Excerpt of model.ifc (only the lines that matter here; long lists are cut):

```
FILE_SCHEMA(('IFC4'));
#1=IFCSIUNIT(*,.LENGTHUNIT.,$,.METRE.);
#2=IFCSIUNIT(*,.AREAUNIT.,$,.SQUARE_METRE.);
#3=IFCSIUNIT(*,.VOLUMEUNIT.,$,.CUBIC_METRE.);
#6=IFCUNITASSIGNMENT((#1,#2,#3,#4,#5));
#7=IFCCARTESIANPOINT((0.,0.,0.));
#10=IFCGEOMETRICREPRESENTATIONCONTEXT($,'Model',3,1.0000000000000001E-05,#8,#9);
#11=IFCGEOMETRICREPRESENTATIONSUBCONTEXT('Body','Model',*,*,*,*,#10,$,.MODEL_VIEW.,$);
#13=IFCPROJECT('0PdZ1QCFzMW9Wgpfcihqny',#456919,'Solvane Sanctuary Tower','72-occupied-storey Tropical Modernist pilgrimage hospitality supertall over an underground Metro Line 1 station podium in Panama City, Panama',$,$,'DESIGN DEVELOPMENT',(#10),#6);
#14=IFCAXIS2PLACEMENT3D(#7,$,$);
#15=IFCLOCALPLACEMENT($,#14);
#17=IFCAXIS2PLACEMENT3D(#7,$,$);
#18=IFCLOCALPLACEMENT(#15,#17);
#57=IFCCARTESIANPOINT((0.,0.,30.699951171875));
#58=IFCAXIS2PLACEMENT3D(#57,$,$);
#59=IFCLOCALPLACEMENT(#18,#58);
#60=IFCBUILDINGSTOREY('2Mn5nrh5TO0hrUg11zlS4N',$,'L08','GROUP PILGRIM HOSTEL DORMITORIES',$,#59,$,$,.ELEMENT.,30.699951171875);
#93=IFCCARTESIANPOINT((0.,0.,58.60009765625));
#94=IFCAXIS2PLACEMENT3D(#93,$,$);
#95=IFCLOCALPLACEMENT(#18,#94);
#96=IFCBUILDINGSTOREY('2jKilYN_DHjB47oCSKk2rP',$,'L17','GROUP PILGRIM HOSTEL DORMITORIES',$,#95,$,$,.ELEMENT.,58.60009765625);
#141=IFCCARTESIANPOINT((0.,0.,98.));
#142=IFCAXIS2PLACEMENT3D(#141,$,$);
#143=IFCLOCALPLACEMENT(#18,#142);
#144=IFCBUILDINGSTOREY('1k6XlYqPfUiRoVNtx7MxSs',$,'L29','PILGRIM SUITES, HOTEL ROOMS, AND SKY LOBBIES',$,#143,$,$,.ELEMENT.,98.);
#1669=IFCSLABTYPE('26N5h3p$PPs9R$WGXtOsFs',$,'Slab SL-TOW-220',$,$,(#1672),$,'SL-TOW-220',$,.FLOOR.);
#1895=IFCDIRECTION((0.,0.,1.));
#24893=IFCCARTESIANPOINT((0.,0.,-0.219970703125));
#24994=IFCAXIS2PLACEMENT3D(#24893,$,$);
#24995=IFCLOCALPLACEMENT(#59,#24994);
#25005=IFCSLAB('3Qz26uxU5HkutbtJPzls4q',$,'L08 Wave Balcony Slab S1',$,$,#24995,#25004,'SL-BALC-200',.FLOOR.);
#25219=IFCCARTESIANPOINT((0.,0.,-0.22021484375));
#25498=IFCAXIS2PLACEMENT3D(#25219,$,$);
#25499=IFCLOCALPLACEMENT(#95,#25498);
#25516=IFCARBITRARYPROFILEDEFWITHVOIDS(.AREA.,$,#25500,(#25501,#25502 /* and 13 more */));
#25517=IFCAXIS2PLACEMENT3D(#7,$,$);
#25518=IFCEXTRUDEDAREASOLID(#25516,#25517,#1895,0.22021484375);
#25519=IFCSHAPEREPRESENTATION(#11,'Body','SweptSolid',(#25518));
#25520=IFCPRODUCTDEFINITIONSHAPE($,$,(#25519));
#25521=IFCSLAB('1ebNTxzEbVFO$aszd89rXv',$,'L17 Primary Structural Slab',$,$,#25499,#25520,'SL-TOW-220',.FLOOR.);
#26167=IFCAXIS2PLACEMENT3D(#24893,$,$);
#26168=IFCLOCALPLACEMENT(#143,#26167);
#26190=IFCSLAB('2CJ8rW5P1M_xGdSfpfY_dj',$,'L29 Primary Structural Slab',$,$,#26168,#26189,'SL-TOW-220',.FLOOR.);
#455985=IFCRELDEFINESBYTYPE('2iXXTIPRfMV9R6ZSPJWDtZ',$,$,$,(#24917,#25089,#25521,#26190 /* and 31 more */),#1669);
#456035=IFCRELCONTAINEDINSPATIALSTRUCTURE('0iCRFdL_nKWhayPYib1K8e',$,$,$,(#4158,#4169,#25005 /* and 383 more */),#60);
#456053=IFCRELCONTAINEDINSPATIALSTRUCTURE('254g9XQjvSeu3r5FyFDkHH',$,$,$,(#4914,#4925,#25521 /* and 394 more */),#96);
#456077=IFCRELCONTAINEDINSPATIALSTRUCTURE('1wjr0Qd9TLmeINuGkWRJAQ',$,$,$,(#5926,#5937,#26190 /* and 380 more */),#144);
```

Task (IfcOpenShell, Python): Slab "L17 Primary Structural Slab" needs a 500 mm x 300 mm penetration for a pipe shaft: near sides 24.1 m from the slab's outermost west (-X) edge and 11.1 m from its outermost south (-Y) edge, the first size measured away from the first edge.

```python
import numpy as np
import ifcopenshell
import ifcopenshell.api.feature
import ifcopenshell.api.geometry
import ifcopenshell.api.root
import ifcopenshell.geom
import ifcopenshell.util.placement
import ifcopenshell.util.representation
import ifcopenshell.util.shape
import ifcopenshell.util.unit

model = ifcopenshell.open("model.ifc")
unit_scale = ifcopenshell.util.unit.calculate_unit_scale(model)
settings = ifcopenshell.geom.settings()


def volume(element):
    """Net volume in cubic metres, openings subtracted."""
    shape = ifcopenshell.geom.create_shape(settings, element)
    return ifcopenshell.util.shape.get_volume(shape.geometry)


slab = model.by_guid("1ebNTxzEbVFO$aszd89rXv")
before = volume(slab)

# Extent in the slab's own axes, in metres. The edges named are its -X and -Y sides.
slab_shape = ifcopenshell.geom.create_shape(settings, slab)
vertices = ifcopenshell.util.shape.get_vertices(slab_shape.geometry)
x_min, y_min, bottom = vertices.min(axis=0)
top = vertices[:, 2].max()

opening = ifcopenshell.api.root.create_entity(model, ifc_class="IfcOpeningElement", name="Pipe shaft opening", predefined_type="OPENING")
context = ifcopenshell.util.representation.get_context(model, "Model", "Body", "MODEL_VIEW")
width, depth = 0.5, 0.3
outline = [(0.0, 0.0), (width, 0.0), (width, depth), (0.0, depth), (0.0, 0.0)]
# Overshoot both faces by 50 mm so the cut is clean.
shape = ifcopenshell.api.geometry.add_slab_representation(
    model, context=context, depth=top - bottom + 0.1, polyline=outline
)
ifcopenshell.api.geometry.assign_representation(model, product=opening, representation=shape)

matrix = ifcopenshell.util.placement.get_local_placement(slab.ObjectPlacement)
matrix[:, 3] = matrix @ np.append(np.array([x_min + 24.1, y_min + 11.1, bottom - 0.05]) / unit_scale, 1.0)
ifcopenshell.api.geometry.edit_object_placement(model, product=opening, matrix=matrix, is_si=False)
ifcopenshell.api.feature.add_feature(model, feature=opening, element=slab)

after = volume(slab)

print(f"slab volume {before:.3f} -> {after:.3f} m3")

model.write("model-out.ifc")
```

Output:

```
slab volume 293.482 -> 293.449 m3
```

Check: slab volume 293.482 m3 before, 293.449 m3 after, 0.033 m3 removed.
